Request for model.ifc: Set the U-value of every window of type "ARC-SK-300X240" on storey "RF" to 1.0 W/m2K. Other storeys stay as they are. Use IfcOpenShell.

First a look at what the model holds.

```python
import ifcopenshell
import ifcopenshell.util.element

model = ifcopenshell.open("model.ifc")
print(model.schema)
storey = next(s for s in model.by_type("IfcBuildingStorey") if s.Name == "RF")
windows = [e for e in ifcopenshell.util.element.get_decomposition(storey) if e.is_a("IfcWindow")]
seen = {}
for e in windows:
    element_type = ifcopenshell.util.element.get_type(e)
    key = (element_type.Name if element_type != e and element_type else None, ifcopenshell.util.element.get_pset(e, "Pset_WindowCommon", "ThermalTransmittance"))
    seen[key] = seen.get(key, 0) + 1
for (name, value), count in sorted(seen.items(), key=str):
    print(count, "x", name, "|", value)
```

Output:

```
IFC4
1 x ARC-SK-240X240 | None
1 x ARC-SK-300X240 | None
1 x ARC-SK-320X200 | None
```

```python
import ifcopenshell
import ifcopenshell.api.pset
import ifcopenshell.util.element

model = ifcopenshell.open("model.ifc")

storey = next(s for s in model.by_type("IfcBuildingStorey") if s.Name == "RF")
windows = [e for e in ifcopenshell.util.element.get_decomposition(storey) if e.is_a("IfcWindow")]

count = 0
for e in windows:
    element_type = ifcopenshell.util.element.get_type(e)
    if element_type in (None, e) or element_type.Name != "ARC-SK-300X240":
        continue
    # add_pset returns the element's existing set when there is one.
    pset = ifcopenshell.api.pset.add_pset(model, product=e, name="Pset_WindowCommon")
    ifcopenshell.api.pset.edit_pset(model, pset=pset, properties={"ThermalTransmittance": 1.0})
    count += 1

print(count, "windows updated")

model.write("model_v2.ifc")
```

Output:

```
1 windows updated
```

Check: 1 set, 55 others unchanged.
